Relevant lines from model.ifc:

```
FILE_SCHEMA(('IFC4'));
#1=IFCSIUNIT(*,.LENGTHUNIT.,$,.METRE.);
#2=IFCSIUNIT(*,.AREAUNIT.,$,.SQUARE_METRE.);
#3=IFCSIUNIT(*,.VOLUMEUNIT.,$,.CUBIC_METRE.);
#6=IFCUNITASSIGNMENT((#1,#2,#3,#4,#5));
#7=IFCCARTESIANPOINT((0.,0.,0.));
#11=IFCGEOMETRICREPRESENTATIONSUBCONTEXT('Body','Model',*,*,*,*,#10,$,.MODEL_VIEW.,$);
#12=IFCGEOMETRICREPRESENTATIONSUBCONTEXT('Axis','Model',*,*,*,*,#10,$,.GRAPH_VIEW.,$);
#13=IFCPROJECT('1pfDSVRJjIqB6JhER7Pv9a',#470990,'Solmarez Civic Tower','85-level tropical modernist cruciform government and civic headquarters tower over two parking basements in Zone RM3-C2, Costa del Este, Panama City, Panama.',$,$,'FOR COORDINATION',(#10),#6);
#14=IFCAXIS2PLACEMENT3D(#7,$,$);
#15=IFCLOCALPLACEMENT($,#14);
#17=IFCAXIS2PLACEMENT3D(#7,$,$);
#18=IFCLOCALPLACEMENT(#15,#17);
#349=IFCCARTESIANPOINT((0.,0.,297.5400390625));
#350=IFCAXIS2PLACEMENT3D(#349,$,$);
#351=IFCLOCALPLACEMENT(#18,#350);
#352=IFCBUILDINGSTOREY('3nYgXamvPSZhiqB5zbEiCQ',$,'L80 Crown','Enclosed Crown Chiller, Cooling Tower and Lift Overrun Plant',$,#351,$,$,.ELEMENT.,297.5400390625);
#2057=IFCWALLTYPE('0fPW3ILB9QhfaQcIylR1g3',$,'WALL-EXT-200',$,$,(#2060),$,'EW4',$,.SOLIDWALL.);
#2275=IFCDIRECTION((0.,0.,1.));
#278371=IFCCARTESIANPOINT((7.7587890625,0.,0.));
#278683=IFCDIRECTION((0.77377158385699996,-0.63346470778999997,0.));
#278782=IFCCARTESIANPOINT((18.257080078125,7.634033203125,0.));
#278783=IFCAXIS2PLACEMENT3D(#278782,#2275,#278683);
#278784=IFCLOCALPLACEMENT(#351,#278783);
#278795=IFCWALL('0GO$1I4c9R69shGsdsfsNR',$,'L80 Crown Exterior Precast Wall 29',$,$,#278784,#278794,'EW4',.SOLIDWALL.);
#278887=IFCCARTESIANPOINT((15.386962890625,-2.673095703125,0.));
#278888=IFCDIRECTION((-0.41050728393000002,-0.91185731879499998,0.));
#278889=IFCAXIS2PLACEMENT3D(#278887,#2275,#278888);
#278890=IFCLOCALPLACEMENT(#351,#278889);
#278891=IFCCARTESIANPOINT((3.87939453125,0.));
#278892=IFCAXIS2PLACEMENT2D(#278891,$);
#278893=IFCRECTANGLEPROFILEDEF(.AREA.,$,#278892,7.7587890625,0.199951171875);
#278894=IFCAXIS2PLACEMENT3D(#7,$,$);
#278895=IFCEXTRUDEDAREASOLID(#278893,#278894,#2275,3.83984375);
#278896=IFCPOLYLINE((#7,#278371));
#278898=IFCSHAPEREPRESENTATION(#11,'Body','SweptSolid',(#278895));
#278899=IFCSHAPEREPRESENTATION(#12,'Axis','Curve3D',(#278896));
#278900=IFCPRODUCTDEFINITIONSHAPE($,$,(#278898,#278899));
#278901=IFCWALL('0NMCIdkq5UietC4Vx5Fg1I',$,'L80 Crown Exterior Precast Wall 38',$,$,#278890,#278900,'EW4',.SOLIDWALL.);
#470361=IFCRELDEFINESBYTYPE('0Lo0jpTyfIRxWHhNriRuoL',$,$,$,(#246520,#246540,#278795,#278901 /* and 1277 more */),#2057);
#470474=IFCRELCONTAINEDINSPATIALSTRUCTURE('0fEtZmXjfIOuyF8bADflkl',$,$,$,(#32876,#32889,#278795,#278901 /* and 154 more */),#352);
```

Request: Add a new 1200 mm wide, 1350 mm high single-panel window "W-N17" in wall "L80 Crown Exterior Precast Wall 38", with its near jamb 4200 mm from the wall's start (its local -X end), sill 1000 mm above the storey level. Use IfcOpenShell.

```python
import numpy as np
import ifcopenshell
import ifcopenshell.api.feature
import ifcopenshell.api.geometry
import ifcopenshell.api.root
import ifcopenshell.api.spatial
import ifcopenshell.geom
import ifcopenshell.util.element
import ifcopenshell.util.placement
import ifcopenshell.util.representation
import ifcopenshell.util.shape
import ifcopenshell.util.unit

model = ifcopenshell.open("model.ifc")
unit_scale = ifcopenshell.util.unit.calculate_unit_scale(model)
settings = ifcopenshell.geom.settings()


def volume(element):
    """Net volume in cubic metres, openings subtracted."""
    shape = ifcopenshell.geom.create_shape(settings, element)
    return ifcopenshell.util.shape.get_volume(shape.geometry)


wall = model.by_guid("0NMCIdkq5UietC4Vx5Fg1I")
storey = ifcopenshell.util.element.get_container(wall, ifc_class="IfcBuildingStorey")
context = ifcopenshell.util.representation.get_context(model, "Model", "Body", "MODEL_VIEW")
before = volume(wall)

width, height, from_end, sill = 1.2, 1.35, 4.2, 1  # metres

# The wall runs along its own X axis, and the end named is its -X end.
wall_shape = ifcopenshell.geom.create_shape(settings, wall)
x, y, z = ifcopenshell.util.shape.get_vertices(wall_shape.geometry).T
start = x.min() + from_end
face, thickness = float(y.min()), float(y.max() - y.min())
wall_matrix = ifcopenshell.util.placement.get_local_placement(wall.ObjectPlacement)
level = ifcopenshell.util.placement.get_local_placement(storey.ObjectPlacement)[2, 3]


def in_wall(x, y):
    """Placement at x, y metres in the wall's axes, at sill height."""
    matrix = wall_matrix.copy()
    matrix[:, 3] = wall_matrix @ np.array([x / unit_scale, y / unit_scale, 0.0, 1.0])
    matrix[2, 3] = level + sill / unit_scale
    return matrix


# Opening: a box that overshoots both wall faces by 50 mm.
opening = ifcopenshell.api.root.create_entity(model, ifc_class="IfcOpeningElement", predefined_type="OPENING")
box = ifcopenshell.api.geometry.add_wall_representation(
    model, context=context, length=width, height=height, thickness=thickness + 0.1
)
ifcopenshell.api.geometry.assign_representation(model, product=opening, representation=box)
ifcopenshell.api.geometry.edit_object_placement(model, product=opening, matrix=in_wall(start, face - 0.05), is_si=False)
ifcopenshell.api.feature.add_feature(model, feature=opening, element=wall)

window = ifcopenshell.api.root.create_entity(model, ifc_class="IfcWindow", name="W-N17", predefined_type="WINDOW")
window.OverallWidth, window.OverallHeight = width / unit_scale, height / unit_scale
window.PartitioningType = "SINGLE_PANEL"
body = ifcopenshell.api.geometry.add_window_representation(
    model,
    context=context,
    overall_width=window.OverallWidth,
    overall_height=window.OverallHeight,
    partition_type="SINGLE_PANEL",
)
ifcopenshell.api.geometry.assign_representation(model, product=window, representation=body)
ifcopenshell.api.spatial.assign_container(model, products=[window], relating_structure=storey)
ifcopenshell.api.feature.add_filling(model, opening=opening, element=window)

# Centre the window in the wall's thickness.
ifcopenshell.api.geometry.edit_object_placement(model, product=window, matrix=in_wall(start, face), is_si=False)
window_shape = ifcopenshell.geom.create_shape(settings, window)
depth = ifcopenshell.util.shape.get_vertices(window_shape.geometry)[:, 1]
offset = face + thickness / 2 - (depth.min() + depth.max()) / 2
ifcopenshell.api.geometry.edit_object_placement(model, product=window, matrix=in_wall(start, offset), is_si=False)

after = volume(wall)

print(f"wall volume {before:.3f} -> {after:.3f} m3")

model.write("model_rev.ifc")
```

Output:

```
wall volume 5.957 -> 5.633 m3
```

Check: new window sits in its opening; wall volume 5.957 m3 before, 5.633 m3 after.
